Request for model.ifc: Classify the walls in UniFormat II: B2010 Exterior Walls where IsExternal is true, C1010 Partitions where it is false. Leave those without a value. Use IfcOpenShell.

First a look at what the model holds.

```python
import ifcopenshell
import ifcopenshell.util.element

model = ifcopenshell.open("model.ifc")
print(model.schema)
print("classifications:", [c.Name for c in model.by_type("IfcClassification")])
values = [ifcopenshell.util.element.get_pset(e, "Pset_WallCommon", "IsExternal") for e in model.by_type("IfcWall")]
for value in (True, False, None):
    print("IsExternal", value, values.count(value))
```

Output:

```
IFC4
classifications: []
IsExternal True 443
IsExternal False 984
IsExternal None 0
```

```python
import ifcopenshell
import ifcopenshell.api.classification
import ifcopenshell.util.element

model = ifcopenshell.open("model.ifc")

system = ifcopenshell.api.classification.add_classification(model, classification="UniFormat II")

walls = model.by_type("IfcWall")
external = {e: ifcopenshell.util.element.get_pset(e, "Pset_WallCommon", "IsExternal") for e in walls}
for flag, code, name in ((True, "B2010", "Exterior Walls"), (False, "C1010", "Partitions")):
    products = [e for e in walls if external[e] is flag]
    ifcopenshell.api.classification.add_reference(
        model, products=products, classification=system, identification=code, name=name
    )
    print(code, len(products))

model.write("model_rev.ifc")
```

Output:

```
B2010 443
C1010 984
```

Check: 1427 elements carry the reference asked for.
